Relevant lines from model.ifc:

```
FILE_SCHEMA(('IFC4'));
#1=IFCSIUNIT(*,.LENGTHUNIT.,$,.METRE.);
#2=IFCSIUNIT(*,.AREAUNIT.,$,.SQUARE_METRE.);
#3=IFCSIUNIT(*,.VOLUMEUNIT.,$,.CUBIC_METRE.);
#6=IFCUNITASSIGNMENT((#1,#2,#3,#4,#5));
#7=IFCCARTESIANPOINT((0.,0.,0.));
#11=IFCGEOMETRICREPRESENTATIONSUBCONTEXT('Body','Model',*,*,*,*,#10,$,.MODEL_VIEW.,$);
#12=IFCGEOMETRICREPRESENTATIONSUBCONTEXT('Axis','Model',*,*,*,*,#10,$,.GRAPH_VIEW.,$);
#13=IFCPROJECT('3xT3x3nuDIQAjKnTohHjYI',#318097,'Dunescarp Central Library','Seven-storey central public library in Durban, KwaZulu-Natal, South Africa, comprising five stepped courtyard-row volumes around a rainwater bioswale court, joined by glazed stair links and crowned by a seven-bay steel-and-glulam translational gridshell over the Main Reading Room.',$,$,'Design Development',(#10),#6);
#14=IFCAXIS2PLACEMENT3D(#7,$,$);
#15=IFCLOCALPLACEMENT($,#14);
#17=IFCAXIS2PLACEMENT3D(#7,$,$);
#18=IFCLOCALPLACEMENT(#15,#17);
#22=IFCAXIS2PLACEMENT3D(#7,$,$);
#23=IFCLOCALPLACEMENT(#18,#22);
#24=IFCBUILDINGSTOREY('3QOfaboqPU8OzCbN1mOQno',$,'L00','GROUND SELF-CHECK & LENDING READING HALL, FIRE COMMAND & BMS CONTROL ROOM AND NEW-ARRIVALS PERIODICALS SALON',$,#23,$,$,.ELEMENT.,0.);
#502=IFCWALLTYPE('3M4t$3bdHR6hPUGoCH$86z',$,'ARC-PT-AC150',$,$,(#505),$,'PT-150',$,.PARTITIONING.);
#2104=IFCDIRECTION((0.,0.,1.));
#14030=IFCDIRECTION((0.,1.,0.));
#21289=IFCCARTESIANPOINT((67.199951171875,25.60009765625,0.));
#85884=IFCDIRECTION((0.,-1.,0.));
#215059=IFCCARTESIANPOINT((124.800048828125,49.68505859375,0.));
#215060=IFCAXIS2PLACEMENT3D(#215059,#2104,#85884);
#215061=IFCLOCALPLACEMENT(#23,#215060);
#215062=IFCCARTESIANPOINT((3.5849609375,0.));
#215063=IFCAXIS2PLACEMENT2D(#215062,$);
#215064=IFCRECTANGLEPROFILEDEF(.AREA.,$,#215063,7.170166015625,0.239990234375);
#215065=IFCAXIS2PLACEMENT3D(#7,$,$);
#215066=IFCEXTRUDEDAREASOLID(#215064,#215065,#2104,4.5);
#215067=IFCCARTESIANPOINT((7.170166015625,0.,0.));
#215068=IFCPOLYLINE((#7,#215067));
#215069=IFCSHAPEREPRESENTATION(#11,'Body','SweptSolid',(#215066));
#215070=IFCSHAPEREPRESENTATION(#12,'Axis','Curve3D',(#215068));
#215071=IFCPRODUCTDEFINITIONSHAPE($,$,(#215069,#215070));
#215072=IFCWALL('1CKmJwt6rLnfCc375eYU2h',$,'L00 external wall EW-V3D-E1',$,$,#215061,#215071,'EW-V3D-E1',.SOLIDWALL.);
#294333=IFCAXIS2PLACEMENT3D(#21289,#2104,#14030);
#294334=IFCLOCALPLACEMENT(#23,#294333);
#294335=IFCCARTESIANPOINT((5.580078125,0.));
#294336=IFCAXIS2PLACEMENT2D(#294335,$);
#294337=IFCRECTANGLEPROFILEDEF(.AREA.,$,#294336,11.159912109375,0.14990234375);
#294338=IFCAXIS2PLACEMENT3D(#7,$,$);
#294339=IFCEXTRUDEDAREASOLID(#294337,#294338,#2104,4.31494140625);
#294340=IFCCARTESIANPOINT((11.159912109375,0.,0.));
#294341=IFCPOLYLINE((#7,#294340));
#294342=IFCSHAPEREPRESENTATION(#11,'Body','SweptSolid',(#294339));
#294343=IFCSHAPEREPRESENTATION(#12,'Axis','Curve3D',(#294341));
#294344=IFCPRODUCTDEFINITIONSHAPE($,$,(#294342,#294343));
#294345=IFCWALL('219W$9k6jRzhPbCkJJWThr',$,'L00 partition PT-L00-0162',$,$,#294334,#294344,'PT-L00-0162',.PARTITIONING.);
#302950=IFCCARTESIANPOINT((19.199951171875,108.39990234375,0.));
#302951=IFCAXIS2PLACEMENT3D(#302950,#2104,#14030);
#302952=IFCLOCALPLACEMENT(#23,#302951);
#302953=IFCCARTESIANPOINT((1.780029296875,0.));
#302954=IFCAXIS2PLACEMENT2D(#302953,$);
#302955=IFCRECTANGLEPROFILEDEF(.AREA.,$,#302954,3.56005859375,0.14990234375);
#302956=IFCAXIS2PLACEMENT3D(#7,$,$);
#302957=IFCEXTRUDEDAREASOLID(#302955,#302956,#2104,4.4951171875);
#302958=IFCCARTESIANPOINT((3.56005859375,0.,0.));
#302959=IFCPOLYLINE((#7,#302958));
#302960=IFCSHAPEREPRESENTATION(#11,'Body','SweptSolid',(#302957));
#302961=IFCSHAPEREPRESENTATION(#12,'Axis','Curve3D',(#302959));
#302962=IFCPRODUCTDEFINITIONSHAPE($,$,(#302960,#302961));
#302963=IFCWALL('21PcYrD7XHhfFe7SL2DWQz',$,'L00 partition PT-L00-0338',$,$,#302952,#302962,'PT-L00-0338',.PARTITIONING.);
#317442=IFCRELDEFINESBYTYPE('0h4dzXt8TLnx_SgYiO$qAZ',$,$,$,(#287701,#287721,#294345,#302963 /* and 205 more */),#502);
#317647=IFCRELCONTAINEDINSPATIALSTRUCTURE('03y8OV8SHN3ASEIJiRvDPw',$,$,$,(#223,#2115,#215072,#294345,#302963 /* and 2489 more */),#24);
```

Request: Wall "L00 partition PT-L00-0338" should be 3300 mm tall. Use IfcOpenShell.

```python
import ifcopenshell
import ifcopenshell.geom
import ifcopenshell.util.representation
import ifcopenshell.util.shape
import ifcopenshell.util.unit

model = ifcopenshell.open("model.ifc")
unit_scale = ifcopenshell.util.unit.calculate_unit_scale(model)
settings = ifcopenshell.geom.settings()


def volume(element):
    """Net volume in cubic metres, openings subtracted."""
    shape = ifcopenshell.geom.create_shape(settings, element)
    return ifcopenshell.util.shape.get_volume(shape.geometry)


wall = model.by_id(302963)
before = volume(wall)

body = ifcopenshell.util.representation.get_representation(wall, "Model", "Body")
solid = body.Items[0]
old_height = solid.Depth
solid.Depth = 3.3 / unit_scale
after = volume(wall)

print(f"height {old_height:g} -> {solid.Depth:g}, volume {before:.3f} -> {after:.3f} m3")

model.write("model_updated.ifc")
```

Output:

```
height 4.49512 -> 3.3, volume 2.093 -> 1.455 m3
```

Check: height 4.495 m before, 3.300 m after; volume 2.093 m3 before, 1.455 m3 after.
